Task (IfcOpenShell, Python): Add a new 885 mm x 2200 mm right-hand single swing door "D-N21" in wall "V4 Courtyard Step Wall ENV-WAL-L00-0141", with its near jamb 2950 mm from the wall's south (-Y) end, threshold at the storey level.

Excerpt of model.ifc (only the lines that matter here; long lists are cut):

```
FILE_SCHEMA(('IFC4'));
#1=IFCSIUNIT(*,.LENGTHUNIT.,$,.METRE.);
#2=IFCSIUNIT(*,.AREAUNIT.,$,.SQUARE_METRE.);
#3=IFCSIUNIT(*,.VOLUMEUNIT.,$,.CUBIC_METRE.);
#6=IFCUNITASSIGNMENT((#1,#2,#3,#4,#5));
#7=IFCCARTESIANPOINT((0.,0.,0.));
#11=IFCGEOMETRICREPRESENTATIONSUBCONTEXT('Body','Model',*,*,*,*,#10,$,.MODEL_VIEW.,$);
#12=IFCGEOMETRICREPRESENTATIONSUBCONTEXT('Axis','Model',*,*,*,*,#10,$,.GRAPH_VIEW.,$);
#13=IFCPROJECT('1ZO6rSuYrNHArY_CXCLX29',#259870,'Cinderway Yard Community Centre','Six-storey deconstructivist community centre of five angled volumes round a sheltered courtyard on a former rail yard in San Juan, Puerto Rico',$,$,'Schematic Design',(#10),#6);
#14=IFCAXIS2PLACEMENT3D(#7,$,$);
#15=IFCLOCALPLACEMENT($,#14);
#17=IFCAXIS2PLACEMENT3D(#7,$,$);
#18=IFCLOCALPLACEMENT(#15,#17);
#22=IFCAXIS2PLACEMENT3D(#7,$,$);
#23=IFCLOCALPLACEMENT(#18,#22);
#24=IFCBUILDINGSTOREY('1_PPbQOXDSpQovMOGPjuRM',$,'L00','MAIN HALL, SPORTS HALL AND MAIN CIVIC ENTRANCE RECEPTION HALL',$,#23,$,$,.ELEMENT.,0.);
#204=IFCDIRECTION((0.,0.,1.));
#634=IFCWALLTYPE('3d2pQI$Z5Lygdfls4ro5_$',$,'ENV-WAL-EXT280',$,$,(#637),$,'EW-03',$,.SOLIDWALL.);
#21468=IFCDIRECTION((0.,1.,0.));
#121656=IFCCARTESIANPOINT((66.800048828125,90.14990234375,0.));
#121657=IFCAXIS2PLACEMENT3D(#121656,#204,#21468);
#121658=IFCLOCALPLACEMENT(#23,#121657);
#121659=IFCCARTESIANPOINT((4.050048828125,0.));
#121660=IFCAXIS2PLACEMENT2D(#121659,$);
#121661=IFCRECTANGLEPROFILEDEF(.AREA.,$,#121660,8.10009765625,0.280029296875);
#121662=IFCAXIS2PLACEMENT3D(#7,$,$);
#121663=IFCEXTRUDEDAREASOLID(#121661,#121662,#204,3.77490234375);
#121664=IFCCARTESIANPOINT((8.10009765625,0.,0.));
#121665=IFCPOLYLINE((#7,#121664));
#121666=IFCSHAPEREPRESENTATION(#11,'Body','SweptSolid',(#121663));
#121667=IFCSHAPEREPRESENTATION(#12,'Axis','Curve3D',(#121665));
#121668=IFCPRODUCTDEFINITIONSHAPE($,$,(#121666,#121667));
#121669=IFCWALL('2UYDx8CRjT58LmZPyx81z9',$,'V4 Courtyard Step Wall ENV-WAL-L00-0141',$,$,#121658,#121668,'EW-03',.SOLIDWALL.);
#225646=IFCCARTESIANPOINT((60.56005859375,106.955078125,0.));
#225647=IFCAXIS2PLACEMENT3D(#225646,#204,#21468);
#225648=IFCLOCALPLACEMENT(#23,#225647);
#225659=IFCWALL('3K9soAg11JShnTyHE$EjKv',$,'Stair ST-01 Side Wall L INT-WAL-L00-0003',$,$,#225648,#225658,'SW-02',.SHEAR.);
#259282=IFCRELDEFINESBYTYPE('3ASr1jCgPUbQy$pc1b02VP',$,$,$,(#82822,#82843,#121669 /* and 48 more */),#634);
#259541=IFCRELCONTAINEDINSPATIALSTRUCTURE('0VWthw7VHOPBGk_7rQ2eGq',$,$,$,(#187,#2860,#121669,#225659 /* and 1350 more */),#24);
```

```python
import numpy as np
import ifcopenshell
import ifcopenshell.api.feature
import ifcopenshell.api.geometry
import ifcopenshell.api.root
import ifcopenshell.api.spatial
import ifcopenshell.geom
import ifcopenshell.util.element
import ifcopenshell.util.placement
import ifcopenshell.util.representation
import ifcopenshell.util.shape
import ifcopenshell.util.unit

model = ifcopenshell.open("model.ifc")
unit_scale = ifcopenshell.util.unit.calculate_unit_scale(model)
settings = ifcopenshell.geom.settings()


def volume(element):
    """Net volume in cubic metres, openings subtracted."""
    shape = ifcopenshell.geom.create_shape(settings, element)
    return ifcopenshell.util.shape.get_volume(shape.geometry)


wall = model.by_guid("2UYDx8CRjT58LmZPyx81z9")
storey = ifcopenshell.util.element.get_container(wall, ifc_class="IfcBuildingStorey")
context = ifcopenshell.util.representation.get_context(model, "Model", "Body", "MODEL_VIEW")
before = volume(wall)

width, height, from_end, sill = 0.885, 2.2, 2.95, 0.0  # metres

# The wall runs along its own X axis, and the end named is its -X end.
wall_shape = ifcopenshell.geom.create_shape(settings, wall)
x, y, z = ifcopenshell.util.shape.get_vertices(wall_shape.geometry).T
start = x.min() + from_end
face, thickness = float(y.min()), float(y.max() - y.min())
wall_matrix = ifcopenshell.util.placement.get_local_placement(wall.ObjectPlacement)
level = ifcopenshell.util.placement.get_local_placement(storey.ObjectPlacement)[2, 3]


def in_wall(x, y):
    """Placement at x, y metres in the wall's axes, at sill height."""
    matrix = wall_matrix.copy()
    matrix[:, 3] = wall_matrix @ np.array([x / unit_scale, y / unit_scale, 0.0, 1.0])
    matrix[2, 3] = level + sill / unit_scale
    return matrix


# Opening: a box that overshoots both wall faces by 50 mm.
opening = ifcopenshell.api.root.create_entity(model, ifc_class="IfcOpeningElement", predefined_type="OPENING")
box = ifcopenshell.api.geometry.add_wall_representation(
    model, context=context, length=width, height=height, thickness=thickness + 0.1
)
ifcopenshell.api.geometry.assign_representation(model, product=opening, representation=box)
ifcopenshell.api.geometry.edit_object_placement(model, product=opening, matrix=in_wall(start, face - 0.05), is_si=False)
ifcopenshell.api.feature.add_feature(model, feature=opening, element=wall)

door = ifcopenshell.api.root.create_entity(model, ifc_class="IfcDoor", name="D-N21", predefined_type="DOOR")
door.OverallWidth, door.OverallHeight = width / unit_scale, height / unit_scale
door.OperationType = "SINGLE_SWING_RIGHT"
body = ifcopenshell.api.geometry.add_door_representation(
    model,
    context=context,
    overall_width=door.OverallWidth,
    overall_height=door.OverallHeight,
    operation_type="SINGLE_SWING_RIGHT",
    lining_properties={"LiningDepth": thickness / unit_scale, "ThresholdDepth": thickness / unit_scale},
)
ifcopenshell.api.geometry.assign_representation(model, product=door, representation=body)
ifcopenshell.api.spatial.assign_container(model, products=[door], relating_structure=storey)
ifcopenshell.api.feature.add_filling(model, opening=opening, element=door)

# The lining spans the wall, so the door starts at the wall face.
ifcopenshell.api.geometry.edit_object_placement(model, product=door, matrix=in_wall(start, face), is_si=False)

after = volume(wall)

print(f"wall volume {before:.3f} -> {after:.3f} m3")

model.write("model_edited.ifc")
```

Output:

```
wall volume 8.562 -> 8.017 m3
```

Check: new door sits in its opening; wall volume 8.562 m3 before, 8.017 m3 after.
